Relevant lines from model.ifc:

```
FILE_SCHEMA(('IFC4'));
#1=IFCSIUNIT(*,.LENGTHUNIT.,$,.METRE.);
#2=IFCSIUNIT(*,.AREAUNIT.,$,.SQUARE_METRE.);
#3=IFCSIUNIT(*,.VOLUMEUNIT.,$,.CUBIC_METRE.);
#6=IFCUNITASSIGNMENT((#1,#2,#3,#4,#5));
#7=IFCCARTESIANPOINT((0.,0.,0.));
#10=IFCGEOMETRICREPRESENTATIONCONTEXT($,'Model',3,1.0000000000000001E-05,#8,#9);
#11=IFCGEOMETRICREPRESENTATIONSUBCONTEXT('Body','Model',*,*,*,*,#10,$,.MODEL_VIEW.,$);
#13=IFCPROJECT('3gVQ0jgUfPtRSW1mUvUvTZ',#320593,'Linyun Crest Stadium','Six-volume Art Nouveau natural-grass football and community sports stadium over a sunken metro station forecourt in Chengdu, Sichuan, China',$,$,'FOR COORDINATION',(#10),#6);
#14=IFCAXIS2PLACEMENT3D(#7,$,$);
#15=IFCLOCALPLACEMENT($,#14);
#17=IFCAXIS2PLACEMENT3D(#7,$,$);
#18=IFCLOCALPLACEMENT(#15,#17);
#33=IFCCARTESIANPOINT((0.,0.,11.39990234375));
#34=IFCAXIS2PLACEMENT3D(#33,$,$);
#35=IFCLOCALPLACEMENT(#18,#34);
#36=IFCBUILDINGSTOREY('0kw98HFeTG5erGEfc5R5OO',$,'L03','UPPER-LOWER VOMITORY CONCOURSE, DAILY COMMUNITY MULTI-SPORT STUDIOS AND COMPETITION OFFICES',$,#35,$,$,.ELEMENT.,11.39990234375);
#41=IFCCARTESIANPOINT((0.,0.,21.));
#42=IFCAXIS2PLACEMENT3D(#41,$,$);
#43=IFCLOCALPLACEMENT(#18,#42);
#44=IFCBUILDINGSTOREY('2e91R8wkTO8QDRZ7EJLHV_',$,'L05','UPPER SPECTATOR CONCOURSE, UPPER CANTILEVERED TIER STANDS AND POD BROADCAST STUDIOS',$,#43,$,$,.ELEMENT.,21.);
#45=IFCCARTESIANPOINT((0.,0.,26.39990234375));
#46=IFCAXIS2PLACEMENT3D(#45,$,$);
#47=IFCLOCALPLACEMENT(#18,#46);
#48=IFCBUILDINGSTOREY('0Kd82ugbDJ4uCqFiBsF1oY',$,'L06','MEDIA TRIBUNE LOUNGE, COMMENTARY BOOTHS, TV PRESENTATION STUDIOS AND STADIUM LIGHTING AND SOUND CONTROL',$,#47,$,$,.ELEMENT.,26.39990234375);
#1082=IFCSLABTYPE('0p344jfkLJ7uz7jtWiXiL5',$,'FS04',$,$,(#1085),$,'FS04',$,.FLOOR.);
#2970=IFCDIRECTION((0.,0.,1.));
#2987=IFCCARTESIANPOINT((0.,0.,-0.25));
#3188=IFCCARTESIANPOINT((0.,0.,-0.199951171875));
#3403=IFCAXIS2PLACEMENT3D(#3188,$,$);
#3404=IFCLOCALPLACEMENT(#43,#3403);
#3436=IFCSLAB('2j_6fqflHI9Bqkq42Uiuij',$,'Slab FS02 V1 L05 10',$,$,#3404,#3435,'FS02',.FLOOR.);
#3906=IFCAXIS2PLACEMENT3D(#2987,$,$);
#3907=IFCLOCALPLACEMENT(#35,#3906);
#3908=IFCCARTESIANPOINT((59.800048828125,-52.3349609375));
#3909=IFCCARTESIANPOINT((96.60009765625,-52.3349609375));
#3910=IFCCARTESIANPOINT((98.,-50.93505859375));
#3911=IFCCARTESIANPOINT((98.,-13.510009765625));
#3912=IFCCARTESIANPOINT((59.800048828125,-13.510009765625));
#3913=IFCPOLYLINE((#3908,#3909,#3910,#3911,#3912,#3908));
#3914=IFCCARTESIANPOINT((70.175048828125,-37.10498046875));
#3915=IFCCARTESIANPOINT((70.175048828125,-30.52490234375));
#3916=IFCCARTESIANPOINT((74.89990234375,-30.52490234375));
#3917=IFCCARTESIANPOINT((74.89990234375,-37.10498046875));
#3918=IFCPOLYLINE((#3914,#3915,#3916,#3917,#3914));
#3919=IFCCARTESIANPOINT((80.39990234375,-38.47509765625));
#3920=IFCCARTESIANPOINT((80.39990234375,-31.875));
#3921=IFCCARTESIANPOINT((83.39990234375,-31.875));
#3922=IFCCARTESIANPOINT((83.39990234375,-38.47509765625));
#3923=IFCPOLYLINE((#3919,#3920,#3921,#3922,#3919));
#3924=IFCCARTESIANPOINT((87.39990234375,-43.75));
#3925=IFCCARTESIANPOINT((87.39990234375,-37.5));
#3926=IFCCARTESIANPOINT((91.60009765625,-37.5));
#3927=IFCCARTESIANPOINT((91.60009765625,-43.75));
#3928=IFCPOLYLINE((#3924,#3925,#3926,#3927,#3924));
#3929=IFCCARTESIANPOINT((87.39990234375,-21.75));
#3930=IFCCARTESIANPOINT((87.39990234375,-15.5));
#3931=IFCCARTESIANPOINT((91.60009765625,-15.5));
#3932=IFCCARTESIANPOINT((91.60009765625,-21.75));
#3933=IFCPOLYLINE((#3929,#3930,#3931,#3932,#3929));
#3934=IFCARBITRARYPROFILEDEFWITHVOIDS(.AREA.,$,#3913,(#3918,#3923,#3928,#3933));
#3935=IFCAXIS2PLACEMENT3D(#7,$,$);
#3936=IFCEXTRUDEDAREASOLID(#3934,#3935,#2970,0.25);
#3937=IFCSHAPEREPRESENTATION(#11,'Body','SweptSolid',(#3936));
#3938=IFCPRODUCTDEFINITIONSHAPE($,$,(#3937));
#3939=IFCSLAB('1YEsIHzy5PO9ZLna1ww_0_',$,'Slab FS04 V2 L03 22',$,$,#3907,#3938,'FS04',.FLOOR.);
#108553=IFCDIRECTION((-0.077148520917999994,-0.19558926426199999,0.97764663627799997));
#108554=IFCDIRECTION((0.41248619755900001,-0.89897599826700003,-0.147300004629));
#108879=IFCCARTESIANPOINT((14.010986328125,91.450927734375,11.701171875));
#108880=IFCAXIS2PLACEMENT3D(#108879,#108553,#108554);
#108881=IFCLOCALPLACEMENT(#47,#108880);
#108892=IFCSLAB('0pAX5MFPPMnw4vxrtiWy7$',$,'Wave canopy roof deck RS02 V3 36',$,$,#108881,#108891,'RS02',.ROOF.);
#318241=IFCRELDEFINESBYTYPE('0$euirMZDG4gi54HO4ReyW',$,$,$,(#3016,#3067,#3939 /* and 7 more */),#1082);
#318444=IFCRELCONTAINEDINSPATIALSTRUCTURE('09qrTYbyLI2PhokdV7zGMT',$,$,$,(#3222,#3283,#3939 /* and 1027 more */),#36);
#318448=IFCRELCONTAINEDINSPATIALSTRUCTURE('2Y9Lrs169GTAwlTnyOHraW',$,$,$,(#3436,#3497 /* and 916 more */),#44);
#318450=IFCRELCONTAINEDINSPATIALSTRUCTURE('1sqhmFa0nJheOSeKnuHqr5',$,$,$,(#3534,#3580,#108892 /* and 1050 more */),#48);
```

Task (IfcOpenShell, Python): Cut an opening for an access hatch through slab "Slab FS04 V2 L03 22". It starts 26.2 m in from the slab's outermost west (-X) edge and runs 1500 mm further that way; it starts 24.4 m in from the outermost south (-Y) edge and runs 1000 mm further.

```python
import numpy as np
import ifcopenshell
import ifcopenshell.api.feature
import ifcopenshell.api.geometry
import ifcopenshell.api.root
import ifcopenshell.geom
import ifcopenshell.util.placement
import ifcopenshell.util.representation
import ifcopenshell.util.shape
import ifcopenshell.util.unit

model = ifcopenshell.open("model.ifc")
unit_scale = ifcopenshell.util.unit.calculate_unit_scale(model)
settings = ifcopenshell.geom.settings()


def volume(element):
    """Net volume in cubic metres, openings subtracted."""
    shape = ifcopenshell.geom.create_shape(settings, element)
    return ifcopenshell.util.shape.get_volume(shape.geometry)


slab = model.by_guid("1YEsIHzy5PO9ZLna1ww_0_")
before = volume(slab)

# Extent in the slab's own axes, in metres. The edges named are its -X and -Y sides.
slab_shape = ifcopenshell.geom.create_shape(settings, slab)
vertices = ifcopenshell.util.shape.get_vertices(slab_shape.geometry)
x_min, y_min, bottom = vertices.min(axis=0)
top = vertices[:, 2].max()

opening = ifcopenshell.api.root.create_entity(model, ifc_class="IfcOpeningElement", name="Access hatch opening", predefined_type="OPENING")
context = ifcopenshell.util.representation.get_context(model, "Model", "Body", "MODEL_VIEW")
width, depth = 1.5, 1
outline = [(0.0, 0.0), (width, 0.0), (width, depth), (0.0, depth), (0.0, 0.0)]
# Overshoot both faces by 50 mm so the cut is clean.
shape = ifcopenshell.api.geometry.add_slab_representation(
    model, context=context, depth=top - bottom + 0.1, polyline=outline
)
ifcopenshell.api.geometry.assign_representation(model, product=opening, representation=shape)

matrix = ifcopenshell.util.placement.get_local_placement(slab.ObjectPlacement)
matrix[:, 3] = matrix @ np.append(np.array([x_min + 26.2, y_min + 24.4, bottom - 0.05]) / unit_scale, 1.0)
ifcopenshell.api.geometry.edit_object_placement(model, product=opening, matrix=matrix, is_si=False)
ifcopenshell.api.feature.add_feature(model, feature=opening, element=slab)

after = volume(slab)

print(f"slab volume {before:.3f} -> {after:.3f} m3")

model.write("model-out.ifc")
```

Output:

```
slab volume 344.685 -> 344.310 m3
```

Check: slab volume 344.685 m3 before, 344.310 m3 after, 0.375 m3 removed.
